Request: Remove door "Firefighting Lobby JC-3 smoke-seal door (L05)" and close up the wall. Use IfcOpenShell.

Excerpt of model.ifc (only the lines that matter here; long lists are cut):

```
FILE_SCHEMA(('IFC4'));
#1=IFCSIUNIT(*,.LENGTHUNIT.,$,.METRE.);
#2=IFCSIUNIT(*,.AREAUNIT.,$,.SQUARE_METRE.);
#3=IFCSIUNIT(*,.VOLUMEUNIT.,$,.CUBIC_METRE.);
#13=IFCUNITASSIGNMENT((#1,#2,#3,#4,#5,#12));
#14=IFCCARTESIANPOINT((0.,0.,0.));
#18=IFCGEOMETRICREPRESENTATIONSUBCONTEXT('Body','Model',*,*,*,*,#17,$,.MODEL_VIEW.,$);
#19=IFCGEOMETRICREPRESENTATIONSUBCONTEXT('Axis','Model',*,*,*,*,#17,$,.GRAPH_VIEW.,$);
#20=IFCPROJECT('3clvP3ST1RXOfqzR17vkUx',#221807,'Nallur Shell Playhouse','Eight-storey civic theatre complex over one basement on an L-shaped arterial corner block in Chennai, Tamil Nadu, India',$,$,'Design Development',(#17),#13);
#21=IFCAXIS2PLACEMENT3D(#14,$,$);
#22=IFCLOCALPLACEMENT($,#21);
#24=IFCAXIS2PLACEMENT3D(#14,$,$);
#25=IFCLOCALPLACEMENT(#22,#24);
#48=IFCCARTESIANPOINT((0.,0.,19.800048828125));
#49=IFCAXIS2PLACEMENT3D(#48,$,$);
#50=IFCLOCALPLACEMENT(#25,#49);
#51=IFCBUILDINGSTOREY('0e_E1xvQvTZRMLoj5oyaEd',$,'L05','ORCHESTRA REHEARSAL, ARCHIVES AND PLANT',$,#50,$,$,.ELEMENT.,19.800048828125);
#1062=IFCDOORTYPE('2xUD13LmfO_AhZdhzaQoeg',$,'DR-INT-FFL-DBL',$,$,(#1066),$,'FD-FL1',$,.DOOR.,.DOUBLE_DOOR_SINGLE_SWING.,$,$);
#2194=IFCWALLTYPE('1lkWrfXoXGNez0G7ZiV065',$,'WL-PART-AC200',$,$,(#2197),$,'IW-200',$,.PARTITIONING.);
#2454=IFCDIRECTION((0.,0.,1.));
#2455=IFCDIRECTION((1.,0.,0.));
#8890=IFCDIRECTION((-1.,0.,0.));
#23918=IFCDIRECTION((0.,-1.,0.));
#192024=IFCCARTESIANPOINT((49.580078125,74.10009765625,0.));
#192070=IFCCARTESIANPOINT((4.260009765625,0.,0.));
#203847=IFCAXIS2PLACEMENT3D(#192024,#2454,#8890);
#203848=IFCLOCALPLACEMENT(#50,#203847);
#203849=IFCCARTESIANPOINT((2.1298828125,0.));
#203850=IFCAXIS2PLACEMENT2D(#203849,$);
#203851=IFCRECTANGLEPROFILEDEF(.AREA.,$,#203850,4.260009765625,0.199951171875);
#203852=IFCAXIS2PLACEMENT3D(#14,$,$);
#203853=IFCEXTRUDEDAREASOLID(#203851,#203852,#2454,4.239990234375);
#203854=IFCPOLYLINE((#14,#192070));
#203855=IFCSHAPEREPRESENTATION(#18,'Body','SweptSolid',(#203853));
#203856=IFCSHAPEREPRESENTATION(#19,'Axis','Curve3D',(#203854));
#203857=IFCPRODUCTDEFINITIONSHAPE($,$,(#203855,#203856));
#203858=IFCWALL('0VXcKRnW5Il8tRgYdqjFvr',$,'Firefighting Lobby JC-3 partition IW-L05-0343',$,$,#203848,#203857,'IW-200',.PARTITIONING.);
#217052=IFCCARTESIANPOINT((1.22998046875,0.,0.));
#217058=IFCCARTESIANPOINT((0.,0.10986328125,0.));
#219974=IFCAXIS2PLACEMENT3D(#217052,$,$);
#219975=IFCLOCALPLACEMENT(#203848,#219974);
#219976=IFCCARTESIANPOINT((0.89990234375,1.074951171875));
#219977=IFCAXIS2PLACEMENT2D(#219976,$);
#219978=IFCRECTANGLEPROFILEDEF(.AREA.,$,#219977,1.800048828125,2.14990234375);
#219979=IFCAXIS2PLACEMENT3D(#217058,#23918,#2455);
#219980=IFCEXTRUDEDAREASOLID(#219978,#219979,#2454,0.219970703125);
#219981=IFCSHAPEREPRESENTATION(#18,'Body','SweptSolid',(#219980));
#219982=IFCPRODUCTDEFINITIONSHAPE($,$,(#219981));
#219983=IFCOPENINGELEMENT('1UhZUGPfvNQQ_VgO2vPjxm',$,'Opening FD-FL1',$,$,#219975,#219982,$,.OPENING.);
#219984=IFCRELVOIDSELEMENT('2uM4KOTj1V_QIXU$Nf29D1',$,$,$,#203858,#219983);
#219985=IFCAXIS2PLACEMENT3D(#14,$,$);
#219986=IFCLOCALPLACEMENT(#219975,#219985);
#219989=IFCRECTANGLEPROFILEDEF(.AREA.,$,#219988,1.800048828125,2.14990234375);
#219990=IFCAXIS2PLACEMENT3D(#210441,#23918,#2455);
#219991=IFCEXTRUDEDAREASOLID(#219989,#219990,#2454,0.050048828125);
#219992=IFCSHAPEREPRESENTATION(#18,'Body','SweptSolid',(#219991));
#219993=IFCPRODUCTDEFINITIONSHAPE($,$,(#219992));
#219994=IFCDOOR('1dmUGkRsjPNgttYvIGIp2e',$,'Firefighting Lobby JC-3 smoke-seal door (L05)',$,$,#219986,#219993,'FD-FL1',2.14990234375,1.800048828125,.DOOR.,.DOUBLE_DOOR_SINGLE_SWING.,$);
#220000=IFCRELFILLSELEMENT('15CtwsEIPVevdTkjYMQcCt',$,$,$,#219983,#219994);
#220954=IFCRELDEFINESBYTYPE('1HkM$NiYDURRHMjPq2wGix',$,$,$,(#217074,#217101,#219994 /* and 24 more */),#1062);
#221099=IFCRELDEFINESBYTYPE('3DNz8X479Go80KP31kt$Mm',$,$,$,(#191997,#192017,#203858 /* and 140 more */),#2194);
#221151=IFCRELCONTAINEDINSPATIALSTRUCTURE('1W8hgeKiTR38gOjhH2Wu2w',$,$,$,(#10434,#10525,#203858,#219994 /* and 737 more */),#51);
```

```python
import ifcopenshell
import ifcopenshell.api.feature
import ifcopenshell.api.root
import ifcopenshell.geom
import ifcopenshell.util.shape

model = ifcopenshell.open("model.ifc")
settings = ifcopenshell.geom.settings()


def volume(element):
    """Net volume in cubic metres, openings subtracted."""
    shape = ifcopenshell.geom.create_shape(settings, element)
    return ifcopenshell.util.shape.get_volume(shape.geometry)


door = model.by_guid("1dmUGkRsjPNgttYvIGIp2e")
opening = door.FillsVoids[0].RelatingOpeningElement
wall = opening.VoidsElements[0].RelatingBuildingElement
before = volume(wall)

ifcopenshell.api.root.remove_product(model, product=door)
ifcopenshell.api.feature.remove_feature(model, feature=opening)

after = volume(wall)

print(f"wall volume {before:.3f} -> {after:.3f} m3")

model.write("model_rev.ifc")
```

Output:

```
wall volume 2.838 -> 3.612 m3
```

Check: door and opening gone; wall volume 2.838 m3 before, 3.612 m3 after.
